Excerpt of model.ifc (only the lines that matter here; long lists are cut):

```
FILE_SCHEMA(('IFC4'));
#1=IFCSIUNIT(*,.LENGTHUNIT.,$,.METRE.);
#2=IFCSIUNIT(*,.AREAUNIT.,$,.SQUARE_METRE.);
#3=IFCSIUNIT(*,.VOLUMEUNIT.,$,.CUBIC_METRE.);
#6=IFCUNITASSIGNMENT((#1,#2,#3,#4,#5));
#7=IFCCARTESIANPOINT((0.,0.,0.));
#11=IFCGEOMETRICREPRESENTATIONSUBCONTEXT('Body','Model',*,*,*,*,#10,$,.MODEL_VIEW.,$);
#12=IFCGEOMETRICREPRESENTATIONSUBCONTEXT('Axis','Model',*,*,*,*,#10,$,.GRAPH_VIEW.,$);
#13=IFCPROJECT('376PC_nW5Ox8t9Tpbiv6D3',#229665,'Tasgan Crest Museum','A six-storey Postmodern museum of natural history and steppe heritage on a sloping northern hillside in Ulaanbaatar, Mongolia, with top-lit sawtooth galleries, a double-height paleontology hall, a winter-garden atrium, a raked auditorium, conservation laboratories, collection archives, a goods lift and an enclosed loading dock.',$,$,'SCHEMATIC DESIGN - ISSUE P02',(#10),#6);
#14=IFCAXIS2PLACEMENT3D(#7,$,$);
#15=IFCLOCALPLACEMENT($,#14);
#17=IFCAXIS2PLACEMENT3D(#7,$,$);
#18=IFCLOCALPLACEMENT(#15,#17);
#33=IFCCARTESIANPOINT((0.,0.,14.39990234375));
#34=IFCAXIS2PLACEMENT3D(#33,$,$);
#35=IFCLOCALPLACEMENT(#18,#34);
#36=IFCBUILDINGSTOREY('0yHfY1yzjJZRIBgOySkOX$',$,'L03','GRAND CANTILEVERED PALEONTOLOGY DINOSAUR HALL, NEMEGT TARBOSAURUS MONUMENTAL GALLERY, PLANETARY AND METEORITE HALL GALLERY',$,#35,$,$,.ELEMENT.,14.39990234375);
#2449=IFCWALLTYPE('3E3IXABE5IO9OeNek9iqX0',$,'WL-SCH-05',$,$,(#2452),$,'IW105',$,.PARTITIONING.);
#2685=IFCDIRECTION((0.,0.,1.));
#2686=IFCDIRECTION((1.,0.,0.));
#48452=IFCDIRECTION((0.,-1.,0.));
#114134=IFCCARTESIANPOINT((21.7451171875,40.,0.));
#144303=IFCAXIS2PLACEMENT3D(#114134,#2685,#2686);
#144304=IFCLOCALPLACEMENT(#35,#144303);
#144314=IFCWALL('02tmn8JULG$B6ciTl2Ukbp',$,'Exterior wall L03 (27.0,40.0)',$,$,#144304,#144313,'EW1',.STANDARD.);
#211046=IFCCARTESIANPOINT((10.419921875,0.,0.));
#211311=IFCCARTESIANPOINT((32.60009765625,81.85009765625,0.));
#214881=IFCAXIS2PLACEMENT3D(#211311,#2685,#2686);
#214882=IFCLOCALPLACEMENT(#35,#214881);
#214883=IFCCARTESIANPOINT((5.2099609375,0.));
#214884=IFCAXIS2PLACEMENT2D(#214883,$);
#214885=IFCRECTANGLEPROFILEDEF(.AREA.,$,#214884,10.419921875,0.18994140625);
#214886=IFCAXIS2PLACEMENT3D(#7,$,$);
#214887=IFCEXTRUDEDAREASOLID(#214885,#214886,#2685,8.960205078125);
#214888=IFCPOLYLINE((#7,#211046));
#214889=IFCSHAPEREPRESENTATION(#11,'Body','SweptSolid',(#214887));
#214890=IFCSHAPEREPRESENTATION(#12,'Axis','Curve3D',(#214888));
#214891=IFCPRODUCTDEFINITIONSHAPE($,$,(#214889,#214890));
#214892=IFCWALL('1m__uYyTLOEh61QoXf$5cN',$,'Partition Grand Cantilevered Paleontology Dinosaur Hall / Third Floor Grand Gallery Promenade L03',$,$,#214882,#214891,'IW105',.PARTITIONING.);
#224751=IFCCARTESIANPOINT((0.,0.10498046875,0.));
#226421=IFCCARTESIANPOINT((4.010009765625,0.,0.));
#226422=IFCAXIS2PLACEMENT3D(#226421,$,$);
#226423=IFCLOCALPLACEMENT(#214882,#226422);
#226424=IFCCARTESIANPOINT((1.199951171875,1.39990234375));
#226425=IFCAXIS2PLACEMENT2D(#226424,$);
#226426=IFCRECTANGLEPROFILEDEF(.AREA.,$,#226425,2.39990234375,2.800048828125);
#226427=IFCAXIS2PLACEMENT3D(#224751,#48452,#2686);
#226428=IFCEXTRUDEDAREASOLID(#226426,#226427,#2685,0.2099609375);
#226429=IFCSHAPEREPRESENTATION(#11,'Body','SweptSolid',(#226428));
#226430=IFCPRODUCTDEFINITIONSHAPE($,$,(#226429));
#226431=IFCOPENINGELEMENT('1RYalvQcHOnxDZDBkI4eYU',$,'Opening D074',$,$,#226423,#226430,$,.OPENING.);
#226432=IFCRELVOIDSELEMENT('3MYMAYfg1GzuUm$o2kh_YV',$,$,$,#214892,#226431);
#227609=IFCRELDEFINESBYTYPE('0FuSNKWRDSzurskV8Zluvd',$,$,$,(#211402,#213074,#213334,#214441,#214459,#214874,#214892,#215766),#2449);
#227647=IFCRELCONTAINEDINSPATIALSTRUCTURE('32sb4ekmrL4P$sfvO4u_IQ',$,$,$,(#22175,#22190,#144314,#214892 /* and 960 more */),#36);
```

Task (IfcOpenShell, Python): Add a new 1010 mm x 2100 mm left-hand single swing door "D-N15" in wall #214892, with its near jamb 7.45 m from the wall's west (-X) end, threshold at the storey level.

```python
import numpy as np
import ifcopenshell
import ifcopenshell.api.feature
import ifcopenshell.api.geometry
import ifcopenshell.api.root
import ifcopenshell.api.spatial
import ifcopenshell.geom
import ifcopenshell.util.element
import ifcopenshell.util.placement
import ifcopenshell.util.representation
import ifcopenshell.util.shape
import ifcopenshell.util.unit

model = ifcopenshell.open("model.ifc")
unit_scale = ifcopenshell.util.unit.calculate_unit_scale(model)
settings = ifcopenshell.geom.settings()


def volume(element):
    """Net volume in cubic metres, openings subtracted."""
    shape = ifcopenshell.geom.create_shape(settings, element)
    return ifcopenshell.util.shape.get_volume(shape.geometry)


wall = model.by_guid("1m__uYyTLOEh61QoXf$5cN")
storey = ifcopenshell.util.element.get_container(wall, ifc_class="IfcBuildingStorey")
context = ifcopenshell.util.representation.get_context(model, "Model", "Body", "MODEL_VIEW")
before = volume(wall)

width, height, from_end, sill = 1.01, 2.1, 7.45, 0.0  # metres

# The wall runs along its own X axis, and the end named is its -X end.
wall_shape = ifcopenshell.geom.create_shape(settings, wall)
x, y, z = ifcopenshell.util.shape.get_vertices(wall_shape.geometry).T
start = x.min() + from_end
face, thickness = float(y.min()), float(y.max() - y.min())
wall_matrix = ifcopenshell.util.placement.get_local_placement(wall.ObjectPlacement)
level = ifcopenshell.util.placement.get_local_placement(storey.ObjectPlacement)[2, 3]


def in_wall(x, y):
    """Placement at x, y metres in the wall's axes, at sill height."""
    matrix = wall_matrix.copy()
    matrix[:, 3] = wall_matrix @ np.array([x / unit_scale, y / unit_scale, 0.0, 1.0])
    matrix[2, 3] = level + sill / unit_scale
    return matrix


# Opening: a box that overshoots both wall faces by 50 mm.
opening = ifcopenshell.api.root.create_entity(model, ifc_class="IfcOpeningElement", predefined_type="OPENING")
box = ifcopenshell.api.geometry.add_wall_representation(
    model, context=context, length=width, height=height, thickness=thickness + 0.1
)
ifcopenshell.api.geometry.assign_representation(model, product=opening, representation=box)
ifcopenshell.api.geometry.edit_object_placement(model, product=opening, matrix=in_wall(start, face - 0.05), is_si=False)
ifcopenshell.api.feature.add_feature(model, feature=opening, element=wall)

door = ifcopenshell.api.root.create_entity(model, ifc_class="IfcDoor", name="D-N15", predefined_type="DOOR")
door.OverallWidth, door.OverallHeight = width / unit_scale, height / unit_scale
door.OperationType = "SINGLE_SWING_LEFT"
body = ifcopenshell.api.geometry.add_door_representation(
    model,
    context=context,
    overall_width=door.OverallWidth,
    overall_height=door.OverallHeight,
    operation_type="SINGLE_SWING_LEFT",
    lining_properties={"LiningDepth": thickness / unit_scale, "ThresholdDepth": thickness / unit_scale},
)
ifcopenshell.api.geometry.assign_representation(model, product=door, representation=body)
ifcopenshell.api.spatial.assign_container(model, products=[door], relating_structure=storey)
ifcopenshell.api.feature.add_filling(model, opening=opening, element=door)

# The lining spans the wall, so the door starts at the wall face.
ifcopenshell.api.geometry.edit_object_placement(model, product=door, matrix=in_wall(start, face), is_si=False)

after = volume(wall)

print(f"wall volume {before:.3f} -> {after:.3f} m3")

model.write("model_v2.ifc")
```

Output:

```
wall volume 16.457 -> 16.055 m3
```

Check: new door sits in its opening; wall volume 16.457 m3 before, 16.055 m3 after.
